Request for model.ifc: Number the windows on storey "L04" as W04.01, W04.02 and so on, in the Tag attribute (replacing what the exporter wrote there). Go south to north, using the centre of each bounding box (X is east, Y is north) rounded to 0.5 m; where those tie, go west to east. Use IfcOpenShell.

First a look at what the model holds.

```python
import ifcopenshell
import ifcopenshell.util.element
import ifcopenshell.util.placement

model = ifcopenshell.open("model.ifc")
print(model.schema)
storey = next(s for s in model.by_type("IfcBuildingStorey") if s.Name == "L04")
windows = [e for e in ifcopenshell.util.element.get_decomposition(storey) if e.is_a("IfcWindow")]
for e in sorted(windows, key=lambda e: e.id()):
    origin = ifcopenshell.util.placement.get_local_placement(e.ObjectPlacement)[:3, 3]
    print(e.id(), e.Tag, e.Name, origin.round(2) + 0.0, sep=" | ")
```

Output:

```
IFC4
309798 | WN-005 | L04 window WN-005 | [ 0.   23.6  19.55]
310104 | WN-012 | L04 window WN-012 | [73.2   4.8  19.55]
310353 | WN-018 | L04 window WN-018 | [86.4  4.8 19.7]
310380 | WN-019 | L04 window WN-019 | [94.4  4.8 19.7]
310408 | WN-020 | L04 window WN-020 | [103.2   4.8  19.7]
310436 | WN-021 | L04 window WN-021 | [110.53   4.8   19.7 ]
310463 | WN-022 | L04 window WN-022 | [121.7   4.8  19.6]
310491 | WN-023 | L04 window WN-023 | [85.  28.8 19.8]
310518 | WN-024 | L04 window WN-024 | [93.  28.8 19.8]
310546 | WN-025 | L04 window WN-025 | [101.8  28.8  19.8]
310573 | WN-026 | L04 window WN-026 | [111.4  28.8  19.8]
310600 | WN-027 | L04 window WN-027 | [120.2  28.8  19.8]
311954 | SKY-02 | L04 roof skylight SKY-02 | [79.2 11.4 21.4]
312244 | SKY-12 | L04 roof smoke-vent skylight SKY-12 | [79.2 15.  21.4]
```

```python
import ifcopenshell
import ifcopenshell.geom
import ifcopenshell.util.element
import ifcopenshell.util.shape

model = ifcopenshell.open("model.ifc")
settings = ifcopenshell.geom.settings()
settings.set("use-world-coords", True)


def centre(element):
    shape = ifcopenshell.geom.create_shape(settings, element)
    return ifcopenshell.util.shape.get_bbox_centroid(shape.geometry)


storey = next(s for s in model.by_type("IfcBuildingStorey") if s.Name == "L04")
windows = [e for e in ifcopenshell.util.element.get_decomposition(storey) if e.is_a("IfcWindow")]

# Insertion points can sit at a corner or the storey origin, so sort by the geometry (in metres).
centres = {e: centre(e) for e in windows}
windows.sort(key=lambda e: (round(centres[e][1] / 0.5), centres[e][0]))

for i, e in enumerate(windows, start=1):
    number = f"W04.{i:02d}"
    e.Tag = number
    print(e.id(), number)

model.write("model_edited.ifc")
```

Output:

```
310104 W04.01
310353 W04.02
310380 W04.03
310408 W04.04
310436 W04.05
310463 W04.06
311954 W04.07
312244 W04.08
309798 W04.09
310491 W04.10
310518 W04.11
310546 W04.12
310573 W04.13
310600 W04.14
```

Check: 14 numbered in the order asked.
